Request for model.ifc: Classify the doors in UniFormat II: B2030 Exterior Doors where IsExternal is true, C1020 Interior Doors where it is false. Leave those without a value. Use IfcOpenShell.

First a look at what the model holds.

```python
import ifcopenshell
import ifcopenshell.util.element

model = ifcopenshell.open("model.ifc")
print(model.schema)
print("classifications:", [c.Name for c in model.by_type("IfcClassification")])
values = [ifcopenshell.util.element.get_pset(e, "Pset_DoorCommon", "IsExternal") for e in model.by_type("IfcDoor")]
for value in (True, False, None):
    print("IsExternal", value, values.count(value))
```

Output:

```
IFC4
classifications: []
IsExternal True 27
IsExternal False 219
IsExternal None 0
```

```python
import ifcopenshell
import ifcopenshell.api.classification
import ifcopenshell.util.element

model = ifcopenshell.open("model.ifc")

system = ifcopenshell.api.classification.add_classification(model, classification="UniFormat II")

doors = model.by_type("IfcDoor")
external = {e: ifcopenshell.util.element.get_pset(e, "Pset_DoorCommon", "IsExternal") for e in doors}
for flag, code, name in ((True, "B2030", "Exterior Doors"), (False, "C1020", "Interior Doors")):
    products = [e for e in doors if external[e] is flag]
    ifcopenshell.api.classification.add_reference(
        model, products=products, classification=system, identification=code, name=name
    )
    print(code, len(products))

model.write("model_v2.ifc")
```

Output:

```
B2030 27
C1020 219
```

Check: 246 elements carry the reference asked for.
